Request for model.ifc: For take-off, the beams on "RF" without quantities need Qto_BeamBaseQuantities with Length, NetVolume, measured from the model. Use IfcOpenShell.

First a look at what the model holds.

```python
import ifcopenshell
import ifcopenshell.util.element
import ifcopenshell.util.unit

model = ifcopenshell.open("model.ifc")
print(model.schema)
for unit_type in ("LENGTHUNIT", "AREAUNIT", "VOLUMEUNIT"):
    print(unit_type, ifcopenshell.util.unit.calculate_unit_scale(model, unit_type))
storey = next(s for s in model.by_type("IfcBuildingStorey") if s.Name == "RF")
beams = [e for e in ifcopenshell.util.element.get_decomposition(storey) if e.is_a("IfcBeam")]
for e in sorted(beams, key=lambda e: e.id()):
    print(e.id(), e.is_a(), e.Name, list(ifcopenshell.util.element.get_psets(e, qtos_only=True)), sep=" | ")
```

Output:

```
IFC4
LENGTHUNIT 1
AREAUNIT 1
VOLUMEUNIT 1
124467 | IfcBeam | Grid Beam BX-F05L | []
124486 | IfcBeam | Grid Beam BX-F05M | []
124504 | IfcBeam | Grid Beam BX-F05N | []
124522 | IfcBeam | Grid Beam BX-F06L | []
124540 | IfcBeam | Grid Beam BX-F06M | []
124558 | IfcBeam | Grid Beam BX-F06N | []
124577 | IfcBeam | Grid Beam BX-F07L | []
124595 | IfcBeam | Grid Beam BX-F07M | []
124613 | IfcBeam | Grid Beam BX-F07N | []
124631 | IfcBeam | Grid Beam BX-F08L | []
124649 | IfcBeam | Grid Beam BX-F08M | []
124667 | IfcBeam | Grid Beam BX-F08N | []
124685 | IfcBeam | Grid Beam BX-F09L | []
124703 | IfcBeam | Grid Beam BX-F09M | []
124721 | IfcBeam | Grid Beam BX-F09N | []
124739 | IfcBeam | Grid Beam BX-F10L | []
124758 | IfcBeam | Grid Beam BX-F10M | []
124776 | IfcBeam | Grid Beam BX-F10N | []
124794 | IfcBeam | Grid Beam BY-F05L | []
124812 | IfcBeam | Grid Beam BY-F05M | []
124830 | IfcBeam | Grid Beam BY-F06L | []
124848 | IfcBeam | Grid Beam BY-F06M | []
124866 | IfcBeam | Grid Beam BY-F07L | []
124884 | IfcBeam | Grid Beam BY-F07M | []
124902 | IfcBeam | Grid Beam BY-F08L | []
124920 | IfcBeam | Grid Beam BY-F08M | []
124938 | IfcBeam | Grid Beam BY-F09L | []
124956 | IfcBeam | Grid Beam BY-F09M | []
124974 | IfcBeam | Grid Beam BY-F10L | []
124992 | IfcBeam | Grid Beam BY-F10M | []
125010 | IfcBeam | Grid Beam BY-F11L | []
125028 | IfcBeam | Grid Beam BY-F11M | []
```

```python
import ifcopenshell
import ifcopenshell.api.pset
import ifcopenshell.geom
import ifcopenshell.util.element
import ifcopenshell.util.shape
import ifcopenshell.util.unit

model = ifcopenshell.open("model.ifc")
unit_scale = ifcopenshell.util.unit.calculate_unit_scale(model)
volume_scale = ifcopenshell.util.unit.calculate_unit_scale(model, "VOLUMEUNIT")
settings = ifcopenshell.geom.settings()

storey = next(s for s in model.by_type("IfcBuildingStorey") if s.Name == "RF")
beams = [e for e in ifcopenshell.util.element.get_decomposition(storey) if e.is_a("IfcBeam")]

for e in sorted(beams, key=lambda e: e.id()):
    if ifcopenshell.util.element.get_psets(e, qtos_only=True, should_inherit=False):
        continue
    # Geometry comes back in metres, in the element's own axes.
    shape = ifcopenshell.geom.create_shape(settings, e)
    values = {
        "Length": ifcopenshell.util.shape.get_max_xyz(shape.geometry) / unit_scale,
        "NetVolume": ifcopenshell.util.shape.get_volume(shape.geometry) / volume_scale,
    }
    qto = ifcopenshell.api.pset.add_qto(model, product=e, name="Qto_BeamBaseQuantities")
    ifcopenshell.api.pset.edit_qto(model, qto=qto, properties=values)
    print(e.id(), {k: round(v, 3) for k, v in values.items()})

model.write("model_edited.ifc")
```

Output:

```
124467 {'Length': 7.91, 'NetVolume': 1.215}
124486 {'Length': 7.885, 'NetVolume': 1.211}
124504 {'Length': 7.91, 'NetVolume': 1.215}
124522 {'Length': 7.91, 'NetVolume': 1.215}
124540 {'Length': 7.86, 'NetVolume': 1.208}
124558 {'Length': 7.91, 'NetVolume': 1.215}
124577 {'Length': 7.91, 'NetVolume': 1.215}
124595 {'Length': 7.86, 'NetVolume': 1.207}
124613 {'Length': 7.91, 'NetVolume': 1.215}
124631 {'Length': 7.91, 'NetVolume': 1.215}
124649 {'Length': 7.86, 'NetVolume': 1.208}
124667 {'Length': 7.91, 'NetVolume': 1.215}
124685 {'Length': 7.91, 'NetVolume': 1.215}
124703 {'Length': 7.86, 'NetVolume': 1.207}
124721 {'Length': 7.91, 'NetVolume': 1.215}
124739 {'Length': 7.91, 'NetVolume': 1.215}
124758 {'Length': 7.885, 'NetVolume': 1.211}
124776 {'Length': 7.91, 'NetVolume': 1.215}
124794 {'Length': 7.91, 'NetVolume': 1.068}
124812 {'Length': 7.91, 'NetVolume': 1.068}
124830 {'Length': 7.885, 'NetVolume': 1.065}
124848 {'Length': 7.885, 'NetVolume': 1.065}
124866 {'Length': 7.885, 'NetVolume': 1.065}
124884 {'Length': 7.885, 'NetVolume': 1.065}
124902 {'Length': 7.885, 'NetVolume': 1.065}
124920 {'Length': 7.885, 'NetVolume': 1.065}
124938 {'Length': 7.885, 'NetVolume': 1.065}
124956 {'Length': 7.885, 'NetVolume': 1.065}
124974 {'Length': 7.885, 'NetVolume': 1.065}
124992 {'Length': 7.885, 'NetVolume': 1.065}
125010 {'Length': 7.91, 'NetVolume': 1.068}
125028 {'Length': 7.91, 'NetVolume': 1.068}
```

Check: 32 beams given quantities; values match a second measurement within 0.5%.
